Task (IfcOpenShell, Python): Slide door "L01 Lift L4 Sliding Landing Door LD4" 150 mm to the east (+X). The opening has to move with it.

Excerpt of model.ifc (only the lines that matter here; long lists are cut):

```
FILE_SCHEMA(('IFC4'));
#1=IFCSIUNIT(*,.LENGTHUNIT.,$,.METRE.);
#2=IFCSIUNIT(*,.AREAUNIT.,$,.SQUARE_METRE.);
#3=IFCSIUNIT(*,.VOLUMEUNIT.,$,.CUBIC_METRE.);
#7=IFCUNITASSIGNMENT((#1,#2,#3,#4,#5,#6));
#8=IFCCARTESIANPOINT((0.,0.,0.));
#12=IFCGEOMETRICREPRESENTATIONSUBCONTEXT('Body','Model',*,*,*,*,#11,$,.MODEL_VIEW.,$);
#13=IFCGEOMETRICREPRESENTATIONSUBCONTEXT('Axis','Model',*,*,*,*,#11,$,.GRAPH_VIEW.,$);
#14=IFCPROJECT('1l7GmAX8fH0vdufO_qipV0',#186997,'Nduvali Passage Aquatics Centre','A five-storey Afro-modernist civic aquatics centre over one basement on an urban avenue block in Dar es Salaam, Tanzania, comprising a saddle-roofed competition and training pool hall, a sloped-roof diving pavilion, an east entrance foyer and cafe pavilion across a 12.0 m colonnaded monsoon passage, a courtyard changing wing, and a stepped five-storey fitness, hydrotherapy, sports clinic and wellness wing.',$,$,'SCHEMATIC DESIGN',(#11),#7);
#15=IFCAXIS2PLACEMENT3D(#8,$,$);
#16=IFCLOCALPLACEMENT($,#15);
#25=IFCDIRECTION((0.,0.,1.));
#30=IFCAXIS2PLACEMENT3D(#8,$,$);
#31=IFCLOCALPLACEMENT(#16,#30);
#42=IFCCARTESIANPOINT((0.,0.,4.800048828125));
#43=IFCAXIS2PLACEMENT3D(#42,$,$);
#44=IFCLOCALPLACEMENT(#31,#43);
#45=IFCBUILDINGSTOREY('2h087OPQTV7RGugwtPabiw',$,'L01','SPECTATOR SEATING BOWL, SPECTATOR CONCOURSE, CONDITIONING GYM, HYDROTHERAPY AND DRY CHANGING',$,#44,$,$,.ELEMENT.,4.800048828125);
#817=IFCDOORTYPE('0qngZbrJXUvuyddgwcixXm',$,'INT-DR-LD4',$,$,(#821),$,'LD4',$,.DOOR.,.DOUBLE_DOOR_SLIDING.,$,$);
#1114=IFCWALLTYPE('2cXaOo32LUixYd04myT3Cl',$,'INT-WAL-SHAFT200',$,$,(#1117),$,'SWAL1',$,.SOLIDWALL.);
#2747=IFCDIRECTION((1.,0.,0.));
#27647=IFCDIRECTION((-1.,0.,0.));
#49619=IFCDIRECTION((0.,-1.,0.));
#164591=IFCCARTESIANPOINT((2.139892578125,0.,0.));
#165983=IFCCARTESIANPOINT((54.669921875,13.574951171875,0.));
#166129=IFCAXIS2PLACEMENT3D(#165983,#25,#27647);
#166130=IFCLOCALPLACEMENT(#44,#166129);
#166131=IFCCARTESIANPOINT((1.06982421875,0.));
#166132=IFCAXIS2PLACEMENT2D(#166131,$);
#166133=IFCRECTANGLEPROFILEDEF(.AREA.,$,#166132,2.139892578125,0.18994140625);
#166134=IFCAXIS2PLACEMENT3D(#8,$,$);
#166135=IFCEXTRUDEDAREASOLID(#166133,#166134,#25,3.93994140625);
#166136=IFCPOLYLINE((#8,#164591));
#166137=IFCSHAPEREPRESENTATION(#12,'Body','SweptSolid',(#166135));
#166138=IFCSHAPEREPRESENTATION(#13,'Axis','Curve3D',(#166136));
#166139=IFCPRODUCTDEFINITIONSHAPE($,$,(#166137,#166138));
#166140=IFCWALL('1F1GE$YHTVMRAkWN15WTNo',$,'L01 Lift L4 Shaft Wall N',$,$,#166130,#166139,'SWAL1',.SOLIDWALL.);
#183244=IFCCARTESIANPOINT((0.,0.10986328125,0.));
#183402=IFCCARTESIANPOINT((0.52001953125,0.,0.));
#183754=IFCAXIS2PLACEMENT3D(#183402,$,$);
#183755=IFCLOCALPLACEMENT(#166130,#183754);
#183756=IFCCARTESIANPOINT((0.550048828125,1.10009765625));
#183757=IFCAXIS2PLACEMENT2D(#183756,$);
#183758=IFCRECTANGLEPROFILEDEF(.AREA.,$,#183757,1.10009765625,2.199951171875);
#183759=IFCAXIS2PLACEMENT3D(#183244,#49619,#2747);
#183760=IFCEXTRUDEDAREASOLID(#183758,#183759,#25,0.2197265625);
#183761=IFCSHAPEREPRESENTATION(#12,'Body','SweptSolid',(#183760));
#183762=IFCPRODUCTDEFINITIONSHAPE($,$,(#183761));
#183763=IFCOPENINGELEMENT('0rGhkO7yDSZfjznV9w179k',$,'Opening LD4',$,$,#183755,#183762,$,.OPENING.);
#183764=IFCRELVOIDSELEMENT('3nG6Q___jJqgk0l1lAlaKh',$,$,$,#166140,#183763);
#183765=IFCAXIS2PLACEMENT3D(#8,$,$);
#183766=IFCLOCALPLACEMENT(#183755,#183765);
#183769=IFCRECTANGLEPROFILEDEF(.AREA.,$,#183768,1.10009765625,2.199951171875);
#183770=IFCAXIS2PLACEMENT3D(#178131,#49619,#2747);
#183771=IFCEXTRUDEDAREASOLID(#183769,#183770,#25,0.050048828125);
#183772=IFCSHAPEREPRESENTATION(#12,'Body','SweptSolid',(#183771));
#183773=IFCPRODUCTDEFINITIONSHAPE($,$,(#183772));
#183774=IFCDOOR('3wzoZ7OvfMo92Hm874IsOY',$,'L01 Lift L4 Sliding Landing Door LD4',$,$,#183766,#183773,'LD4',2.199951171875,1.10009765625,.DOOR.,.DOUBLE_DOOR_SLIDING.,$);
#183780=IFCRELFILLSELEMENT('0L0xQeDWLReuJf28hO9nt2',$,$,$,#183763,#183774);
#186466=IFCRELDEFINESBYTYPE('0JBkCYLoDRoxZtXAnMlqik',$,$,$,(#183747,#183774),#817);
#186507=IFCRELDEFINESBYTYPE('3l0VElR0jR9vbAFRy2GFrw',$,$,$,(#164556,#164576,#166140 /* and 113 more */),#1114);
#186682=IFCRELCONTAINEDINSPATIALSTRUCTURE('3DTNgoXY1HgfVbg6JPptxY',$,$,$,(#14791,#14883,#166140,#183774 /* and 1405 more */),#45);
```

```python
import ifcopenshell
import ifcopenshell.api.geometry
import ifcopenshell.util.placement

model = ifcopenshell.open("model.ifc")

door = model.by_guid("3wzoZ7OvfMo92Hm874IsOY")
opening = door.FillsVoids[0].RelatingOpeningElement
wall = opening.VoidsElements[0].RelatingBuildingElement

wall_matrix = ifcopenshell.util.placement.get_local_placement(wall.ObjectPlacement)
shift = wall_matrix[:3, 0] * -0.15
before = ifcopenshell.util.placement.get_local_placement(door.ObjectPlacement)[:3, 3].copy()

# The door is placed relative to its opening, so it follows when the opening moves.
matrix = ifcopenshell.util.placement.get_local_placement(opening.ObjectPlacement)
matrix[:3, 3] += shift
ifcopenshell.api.geometry.edit_object_placement(
    model, product=opening, matrix=matrix, is_si=False, should_transform_children=True
)

after = ifcopenshell.util.placement.get_local_placement(door.ObjectPlacement)[:3, 3]
print("door moved by", (after - before).round(3) + 0.0)

model.write("model_v2.ifc")
```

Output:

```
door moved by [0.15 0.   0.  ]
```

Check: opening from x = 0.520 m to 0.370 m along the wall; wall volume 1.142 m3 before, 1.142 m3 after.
